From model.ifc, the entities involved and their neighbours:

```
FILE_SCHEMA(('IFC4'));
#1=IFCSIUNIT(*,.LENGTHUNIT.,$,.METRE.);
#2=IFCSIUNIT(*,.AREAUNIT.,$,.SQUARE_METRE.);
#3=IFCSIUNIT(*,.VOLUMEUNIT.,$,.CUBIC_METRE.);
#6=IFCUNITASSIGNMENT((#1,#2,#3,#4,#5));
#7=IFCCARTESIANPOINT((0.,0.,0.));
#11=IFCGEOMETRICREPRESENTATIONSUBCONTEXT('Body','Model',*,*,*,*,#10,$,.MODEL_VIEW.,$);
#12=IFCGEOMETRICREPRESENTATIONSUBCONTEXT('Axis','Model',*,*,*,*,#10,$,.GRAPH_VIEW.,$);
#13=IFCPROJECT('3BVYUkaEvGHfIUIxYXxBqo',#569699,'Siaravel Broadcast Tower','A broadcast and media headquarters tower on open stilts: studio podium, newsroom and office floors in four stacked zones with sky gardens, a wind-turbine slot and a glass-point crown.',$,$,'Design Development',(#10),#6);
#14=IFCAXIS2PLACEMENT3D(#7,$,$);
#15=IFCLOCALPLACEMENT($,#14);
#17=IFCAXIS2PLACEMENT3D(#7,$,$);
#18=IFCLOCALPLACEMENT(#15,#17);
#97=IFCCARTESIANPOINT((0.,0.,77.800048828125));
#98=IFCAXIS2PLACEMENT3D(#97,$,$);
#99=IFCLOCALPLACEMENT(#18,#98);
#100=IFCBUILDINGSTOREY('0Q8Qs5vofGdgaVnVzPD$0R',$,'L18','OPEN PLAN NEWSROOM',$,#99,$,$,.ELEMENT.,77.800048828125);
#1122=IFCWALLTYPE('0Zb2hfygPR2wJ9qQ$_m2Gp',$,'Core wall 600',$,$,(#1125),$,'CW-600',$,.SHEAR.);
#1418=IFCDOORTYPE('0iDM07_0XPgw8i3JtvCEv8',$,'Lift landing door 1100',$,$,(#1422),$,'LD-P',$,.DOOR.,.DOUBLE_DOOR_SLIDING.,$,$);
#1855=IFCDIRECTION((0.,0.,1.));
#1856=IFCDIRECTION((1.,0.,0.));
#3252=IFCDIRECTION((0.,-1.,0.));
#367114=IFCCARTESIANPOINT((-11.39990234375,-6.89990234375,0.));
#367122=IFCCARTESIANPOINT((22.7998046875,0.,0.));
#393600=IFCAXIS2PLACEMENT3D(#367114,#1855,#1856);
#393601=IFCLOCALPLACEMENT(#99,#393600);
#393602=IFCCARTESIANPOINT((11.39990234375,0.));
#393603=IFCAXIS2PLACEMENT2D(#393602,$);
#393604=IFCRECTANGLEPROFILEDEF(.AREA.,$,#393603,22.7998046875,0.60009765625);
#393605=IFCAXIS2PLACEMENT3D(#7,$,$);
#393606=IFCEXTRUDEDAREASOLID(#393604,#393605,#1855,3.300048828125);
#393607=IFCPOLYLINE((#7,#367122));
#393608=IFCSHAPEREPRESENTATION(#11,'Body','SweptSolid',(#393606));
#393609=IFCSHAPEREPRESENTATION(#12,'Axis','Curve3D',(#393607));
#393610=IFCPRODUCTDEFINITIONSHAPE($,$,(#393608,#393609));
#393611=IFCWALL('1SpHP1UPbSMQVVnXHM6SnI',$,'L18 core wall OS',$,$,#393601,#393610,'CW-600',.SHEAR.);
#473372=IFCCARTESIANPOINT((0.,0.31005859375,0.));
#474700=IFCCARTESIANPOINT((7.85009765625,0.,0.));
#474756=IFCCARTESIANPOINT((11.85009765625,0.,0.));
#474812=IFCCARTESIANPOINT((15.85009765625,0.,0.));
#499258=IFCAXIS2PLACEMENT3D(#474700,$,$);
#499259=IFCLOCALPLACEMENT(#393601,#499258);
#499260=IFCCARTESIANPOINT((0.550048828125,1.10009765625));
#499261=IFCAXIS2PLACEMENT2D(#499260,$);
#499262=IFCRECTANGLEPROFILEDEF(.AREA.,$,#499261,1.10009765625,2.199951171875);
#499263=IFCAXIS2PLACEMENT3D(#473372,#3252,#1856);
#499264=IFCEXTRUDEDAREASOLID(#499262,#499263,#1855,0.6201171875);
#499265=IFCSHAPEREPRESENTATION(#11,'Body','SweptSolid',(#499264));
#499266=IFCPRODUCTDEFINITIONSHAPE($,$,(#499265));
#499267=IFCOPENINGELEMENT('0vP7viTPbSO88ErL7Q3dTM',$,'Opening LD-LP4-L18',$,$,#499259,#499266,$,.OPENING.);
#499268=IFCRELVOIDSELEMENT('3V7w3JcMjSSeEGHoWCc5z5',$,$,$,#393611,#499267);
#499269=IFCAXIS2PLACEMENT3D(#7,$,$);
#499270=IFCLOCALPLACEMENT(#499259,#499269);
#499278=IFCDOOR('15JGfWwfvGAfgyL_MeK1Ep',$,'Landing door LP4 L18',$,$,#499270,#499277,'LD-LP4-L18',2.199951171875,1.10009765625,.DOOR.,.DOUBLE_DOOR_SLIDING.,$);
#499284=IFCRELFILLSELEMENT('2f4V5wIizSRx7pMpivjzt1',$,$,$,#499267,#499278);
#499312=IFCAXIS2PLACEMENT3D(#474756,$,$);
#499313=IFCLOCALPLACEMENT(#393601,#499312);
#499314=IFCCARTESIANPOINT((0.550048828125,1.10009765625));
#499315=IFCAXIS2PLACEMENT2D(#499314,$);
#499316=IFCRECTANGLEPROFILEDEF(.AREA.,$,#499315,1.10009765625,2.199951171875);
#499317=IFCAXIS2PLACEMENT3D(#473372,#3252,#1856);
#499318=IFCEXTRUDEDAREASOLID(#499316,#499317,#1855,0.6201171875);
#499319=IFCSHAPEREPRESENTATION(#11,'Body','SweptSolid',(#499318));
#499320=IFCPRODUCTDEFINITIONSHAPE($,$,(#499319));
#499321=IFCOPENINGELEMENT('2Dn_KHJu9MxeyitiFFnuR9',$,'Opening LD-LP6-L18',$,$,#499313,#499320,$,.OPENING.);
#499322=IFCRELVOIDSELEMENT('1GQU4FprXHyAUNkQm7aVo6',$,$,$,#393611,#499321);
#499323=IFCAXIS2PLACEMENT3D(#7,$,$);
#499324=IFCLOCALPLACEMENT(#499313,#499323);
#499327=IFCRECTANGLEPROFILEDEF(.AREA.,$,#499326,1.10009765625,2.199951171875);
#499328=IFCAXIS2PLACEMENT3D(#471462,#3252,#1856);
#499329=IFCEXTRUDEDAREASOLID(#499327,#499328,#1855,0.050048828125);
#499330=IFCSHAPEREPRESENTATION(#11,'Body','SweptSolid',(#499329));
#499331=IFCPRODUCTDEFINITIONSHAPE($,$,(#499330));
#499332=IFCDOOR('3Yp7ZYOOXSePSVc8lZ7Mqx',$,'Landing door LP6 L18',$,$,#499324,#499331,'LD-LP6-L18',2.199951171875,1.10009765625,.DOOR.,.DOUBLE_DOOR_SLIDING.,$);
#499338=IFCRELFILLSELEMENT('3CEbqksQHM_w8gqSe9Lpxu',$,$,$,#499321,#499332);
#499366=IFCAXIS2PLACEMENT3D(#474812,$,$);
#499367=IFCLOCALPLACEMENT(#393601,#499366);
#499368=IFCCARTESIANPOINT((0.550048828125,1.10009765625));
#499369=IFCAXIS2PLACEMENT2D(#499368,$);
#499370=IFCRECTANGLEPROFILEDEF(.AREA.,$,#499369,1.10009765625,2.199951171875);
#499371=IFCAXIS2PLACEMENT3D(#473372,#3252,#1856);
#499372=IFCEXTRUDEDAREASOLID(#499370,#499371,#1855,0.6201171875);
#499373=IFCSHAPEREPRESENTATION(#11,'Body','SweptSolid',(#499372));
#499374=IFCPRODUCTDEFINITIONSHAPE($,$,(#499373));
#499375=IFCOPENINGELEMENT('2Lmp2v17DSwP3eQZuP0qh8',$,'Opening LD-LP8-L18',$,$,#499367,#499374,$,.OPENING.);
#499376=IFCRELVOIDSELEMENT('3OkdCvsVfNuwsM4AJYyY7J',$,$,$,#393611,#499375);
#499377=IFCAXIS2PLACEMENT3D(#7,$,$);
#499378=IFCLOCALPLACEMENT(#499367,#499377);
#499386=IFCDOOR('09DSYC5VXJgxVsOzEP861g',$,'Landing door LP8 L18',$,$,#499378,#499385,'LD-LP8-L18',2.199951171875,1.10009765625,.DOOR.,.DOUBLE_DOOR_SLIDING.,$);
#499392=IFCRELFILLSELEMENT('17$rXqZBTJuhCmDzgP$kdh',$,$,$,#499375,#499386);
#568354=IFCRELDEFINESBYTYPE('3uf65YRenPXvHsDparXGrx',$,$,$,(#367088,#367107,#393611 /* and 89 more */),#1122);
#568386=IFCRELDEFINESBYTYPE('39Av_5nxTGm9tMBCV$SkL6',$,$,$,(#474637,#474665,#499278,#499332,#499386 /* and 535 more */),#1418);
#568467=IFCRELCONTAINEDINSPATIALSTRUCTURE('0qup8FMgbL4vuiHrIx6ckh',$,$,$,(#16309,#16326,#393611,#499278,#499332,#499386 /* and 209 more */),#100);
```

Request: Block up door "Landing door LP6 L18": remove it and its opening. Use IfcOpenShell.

```python
import ifcopenshell
import ifcopenshell.api.feature
import ifcopenshell.api.root
import ifcopenshell.geom
import ifcopenshell.util.shape

model = ifcopenshell.open("model.ifc")
settings = ifcopenshell.geom.settings()


def volume(element):
    """Net volume in cubic metres, openings subtracted."""
    shape = ifcopenshell.geom.create_shape(settings, element)
    return ifcopenshell.util.shape.get_volume(shape.geometry)


door = model.by_guid("3Yp7ZYOOXSePSVc8lZ7Mqx")
opening = door.FillsVoids[0].RelatingOpeningElement
wall = opening.VoidsElements[0].RelatingBuildingElement
before = volume(wall)

ifcopenshell.api.root.remove_product(model, product=door)
ifcopenshell.api.feature.remove_feature(model, feature=opening)

after = volume(wall)

print(f"wall volume {before:.3f} -> {after:.3f} m3")

model.write("model_rev.ifc")
```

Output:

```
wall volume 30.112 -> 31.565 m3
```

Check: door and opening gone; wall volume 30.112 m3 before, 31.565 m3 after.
